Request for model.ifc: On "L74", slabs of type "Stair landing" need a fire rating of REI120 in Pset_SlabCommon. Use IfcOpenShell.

First a look at what the model holds.

```python
import ifcopenshell
import ifcopenshell.util.element

model = ifcopenshell.open("model.ifc")
print(model.schema)
storey = next(s for s in model.by_type("IfcBuildingStorey") if s.Name == "L74")
slabs = [e for e in ifcopenshell.util.element.get_decomposition(storey) if e.is_a("IfcSlab")]
seen = {}
for e in slabs:
    element_type = ifcopenshell.util.element.get_type(e)
    key = (element_type.Name if element_type != e and element_type else None, ifcopenshell.util.element.get_pset(e, "Pset_SlabCommon", "FireRating"))
    seen[key] = seen.get(key, 0) + 1
for (name, value), count in sorted(seen.items(), key=str):
    print(count, "x", name, "|", value)
```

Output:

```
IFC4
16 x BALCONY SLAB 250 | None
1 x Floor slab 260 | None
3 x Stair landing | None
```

```python
import ifcopenshell
import ifcopenshell.api.pset
import ifcopenshell.util.element

model = ifcopenshell.open("model.ifc")

storey = next(s for s in model.by_type("IfcBuildingStorey") if s.Name == "L74")
slabs = [e for e in ifcopenshell.util.element.get_decomposition(storey) if e.is_a("IfcSlab")]

count = 0
for e in slabs:
    element_type = ifcopenshell.util.element.get_type(e)
    if element_type in (None, e) or element_type.Name != "Stair landing":
        continue
    found = ifcopenshell.util.element.get_pset(e, "Pset_SlabCommon", should_inherit=False)
    if found:
        pset = model.by_id(found["id"])
        if len(ifcopenshell.util.element.get_elements_by_pset(pset)) > 1:
            pset = ifcopenshell.api.pset.unshare_pset(model, products=[e], pset=pset)[0]
    else:
        pset = ifcopenshell.api.pset.add_pset(model, product=e, name="Pset_SlabCommon")
    ifcopenshell.api.pset.edit_pset(model, pset=pset, properties={"FireRating": "REI120"})
    count += 1

print(count, "slabs updated")

model.write("model_rev.ifc")
```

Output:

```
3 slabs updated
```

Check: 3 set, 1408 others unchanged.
